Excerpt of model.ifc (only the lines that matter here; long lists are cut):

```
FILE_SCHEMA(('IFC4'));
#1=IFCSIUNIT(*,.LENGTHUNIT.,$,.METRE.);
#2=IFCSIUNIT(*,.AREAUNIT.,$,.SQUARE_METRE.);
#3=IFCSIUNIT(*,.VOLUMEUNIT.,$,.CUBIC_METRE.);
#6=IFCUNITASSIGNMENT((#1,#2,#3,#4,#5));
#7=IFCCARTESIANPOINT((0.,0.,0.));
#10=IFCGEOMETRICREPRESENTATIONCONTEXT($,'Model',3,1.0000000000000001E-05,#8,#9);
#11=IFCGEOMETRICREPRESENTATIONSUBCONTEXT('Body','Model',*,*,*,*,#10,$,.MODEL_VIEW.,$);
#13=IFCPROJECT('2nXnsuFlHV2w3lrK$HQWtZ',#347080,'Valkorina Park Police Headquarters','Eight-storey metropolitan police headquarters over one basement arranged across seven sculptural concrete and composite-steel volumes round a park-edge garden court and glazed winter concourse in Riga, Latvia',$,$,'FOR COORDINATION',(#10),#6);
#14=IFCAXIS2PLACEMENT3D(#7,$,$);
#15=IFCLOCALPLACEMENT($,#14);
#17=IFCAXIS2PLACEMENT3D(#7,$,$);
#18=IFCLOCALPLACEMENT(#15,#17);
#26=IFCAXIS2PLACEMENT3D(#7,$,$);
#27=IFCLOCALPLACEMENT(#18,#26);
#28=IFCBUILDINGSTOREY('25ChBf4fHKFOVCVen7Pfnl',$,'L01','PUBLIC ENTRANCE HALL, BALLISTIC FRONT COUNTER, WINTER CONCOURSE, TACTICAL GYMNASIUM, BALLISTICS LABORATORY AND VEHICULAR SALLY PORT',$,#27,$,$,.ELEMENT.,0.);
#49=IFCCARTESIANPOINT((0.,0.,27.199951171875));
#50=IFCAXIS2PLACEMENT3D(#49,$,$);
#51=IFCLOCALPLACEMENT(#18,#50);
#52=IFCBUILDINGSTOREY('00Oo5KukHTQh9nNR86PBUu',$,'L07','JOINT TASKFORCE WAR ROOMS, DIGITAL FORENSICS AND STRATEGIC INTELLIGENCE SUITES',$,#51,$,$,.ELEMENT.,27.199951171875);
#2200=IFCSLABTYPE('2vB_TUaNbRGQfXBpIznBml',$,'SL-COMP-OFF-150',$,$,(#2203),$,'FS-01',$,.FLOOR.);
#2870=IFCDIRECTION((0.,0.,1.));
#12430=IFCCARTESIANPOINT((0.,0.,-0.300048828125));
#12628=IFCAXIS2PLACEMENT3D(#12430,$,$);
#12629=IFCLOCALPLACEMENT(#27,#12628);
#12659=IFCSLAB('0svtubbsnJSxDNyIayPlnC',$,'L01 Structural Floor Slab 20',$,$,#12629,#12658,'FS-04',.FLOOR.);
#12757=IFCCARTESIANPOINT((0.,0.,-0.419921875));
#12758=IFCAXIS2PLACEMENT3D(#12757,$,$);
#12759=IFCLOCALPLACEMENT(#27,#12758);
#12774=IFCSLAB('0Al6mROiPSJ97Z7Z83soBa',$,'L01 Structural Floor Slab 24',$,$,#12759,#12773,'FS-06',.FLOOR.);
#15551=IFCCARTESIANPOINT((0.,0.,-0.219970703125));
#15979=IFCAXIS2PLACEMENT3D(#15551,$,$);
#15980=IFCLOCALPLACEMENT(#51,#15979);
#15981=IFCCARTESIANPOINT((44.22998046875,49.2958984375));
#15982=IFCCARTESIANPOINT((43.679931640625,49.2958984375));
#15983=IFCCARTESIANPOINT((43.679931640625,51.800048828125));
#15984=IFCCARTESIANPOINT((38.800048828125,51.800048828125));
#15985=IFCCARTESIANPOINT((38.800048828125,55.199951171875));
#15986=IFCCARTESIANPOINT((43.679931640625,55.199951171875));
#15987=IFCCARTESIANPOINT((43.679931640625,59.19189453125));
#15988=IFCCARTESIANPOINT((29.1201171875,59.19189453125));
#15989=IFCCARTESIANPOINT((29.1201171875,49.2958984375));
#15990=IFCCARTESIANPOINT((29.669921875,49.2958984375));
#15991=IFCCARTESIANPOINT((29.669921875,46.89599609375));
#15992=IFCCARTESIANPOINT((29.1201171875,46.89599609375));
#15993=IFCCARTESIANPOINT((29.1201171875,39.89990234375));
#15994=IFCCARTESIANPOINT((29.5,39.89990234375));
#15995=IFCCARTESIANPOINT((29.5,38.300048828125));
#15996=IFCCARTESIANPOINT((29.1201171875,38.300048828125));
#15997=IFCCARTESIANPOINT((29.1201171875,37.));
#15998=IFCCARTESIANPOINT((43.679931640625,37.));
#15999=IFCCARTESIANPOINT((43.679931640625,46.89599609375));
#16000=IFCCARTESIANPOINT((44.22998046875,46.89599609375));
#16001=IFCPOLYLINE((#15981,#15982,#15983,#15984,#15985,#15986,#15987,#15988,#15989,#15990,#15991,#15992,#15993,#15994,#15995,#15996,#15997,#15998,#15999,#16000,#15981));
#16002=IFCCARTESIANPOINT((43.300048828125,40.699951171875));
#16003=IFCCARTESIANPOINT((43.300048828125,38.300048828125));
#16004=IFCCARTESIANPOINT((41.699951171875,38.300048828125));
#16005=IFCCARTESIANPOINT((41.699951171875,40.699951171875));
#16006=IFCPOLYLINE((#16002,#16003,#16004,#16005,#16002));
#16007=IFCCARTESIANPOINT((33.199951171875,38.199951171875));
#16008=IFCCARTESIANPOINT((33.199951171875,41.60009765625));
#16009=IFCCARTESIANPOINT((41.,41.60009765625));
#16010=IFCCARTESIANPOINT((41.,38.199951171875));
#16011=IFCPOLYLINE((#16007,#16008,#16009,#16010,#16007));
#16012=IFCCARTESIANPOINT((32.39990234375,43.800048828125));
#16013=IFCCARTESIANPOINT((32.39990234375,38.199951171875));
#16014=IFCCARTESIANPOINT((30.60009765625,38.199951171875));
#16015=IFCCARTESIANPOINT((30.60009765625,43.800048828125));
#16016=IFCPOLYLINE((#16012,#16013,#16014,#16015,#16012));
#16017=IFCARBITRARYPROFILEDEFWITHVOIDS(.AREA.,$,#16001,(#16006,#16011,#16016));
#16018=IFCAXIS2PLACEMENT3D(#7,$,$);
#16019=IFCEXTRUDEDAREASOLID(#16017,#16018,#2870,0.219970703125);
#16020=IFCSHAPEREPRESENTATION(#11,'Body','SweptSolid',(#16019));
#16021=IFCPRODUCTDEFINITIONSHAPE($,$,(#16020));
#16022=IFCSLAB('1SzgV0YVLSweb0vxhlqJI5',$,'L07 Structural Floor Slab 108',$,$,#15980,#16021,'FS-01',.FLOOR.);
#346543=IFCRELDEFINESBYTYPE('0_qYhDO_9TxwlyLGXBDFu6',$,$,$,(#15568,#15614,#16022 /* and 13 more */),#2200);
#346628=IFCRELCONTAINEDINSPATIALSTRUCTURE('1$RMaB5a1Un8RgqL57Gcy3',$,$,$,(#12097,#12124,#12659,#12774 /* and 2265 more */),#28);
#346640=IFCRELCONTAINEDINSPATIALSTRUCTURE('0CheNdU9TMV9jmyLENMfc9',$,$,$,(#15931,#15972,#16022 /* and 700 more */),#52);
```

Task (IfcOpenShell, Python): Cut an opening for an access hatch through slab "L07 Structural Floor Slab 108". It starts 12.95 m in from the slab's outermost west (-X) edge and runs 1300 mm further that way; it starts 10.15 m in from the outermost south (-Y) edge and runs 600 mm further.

```python
import numpy as np
import ifcopenshell
import ifcopenshell.api.feature
import ifcopenshell.api.geometry
import ifcopenshell.api.root
import ifcopenshell.geom
import ifcopenshell.util.placement
import ifcopenshell.util.representation
import ifcopenshell.util.shape
import ifcopenshell.util.unit

model = ifcopenshell.open("model.ifc")
unit_scale = ifcopenshell.util.unit.calculate_unit_scale(model)
settings = ifcopenshell.geom.settings()


def volume(element):
    """Net volume in cubic metres, openings subtracted."""
    shape = ifcopenshell.geom.create_shape(settings, element)
    return ifcopenshell.util.shape.get_volume(shape.geometry)


slab = model.by_guid("1SzgV0YVLSweb0vxhlqJI5")
before = volume(slab)

# Extent in the slab's own axes, in metres. The edges named are its -X and -Y sides.
slab_shape = ifcopenshell.geom.create_shape(settings, slab)
vertices = ifcopenshell.util.shape.get_vertices(slab_shape.geometry)
x_min, y_min, bottom = vertices.min(axis=0)
top = vertices[:, 2].max()

opening = ifcopenshell.api.root.create_entity(model, ifc_class="IfcOpeningElement", name="Access hatch opening", predefined_type="OPENING")
context = ifcopenshell.util.representation.get_context(model, "Model", "Body", "MODEL_VIEW")
width, depth = 1.3, 0.6
outline = [(0.0, 0.0), (width, 0.0), (width, depth), (0.0, depth), (0.0, 0.0)]
# Overshoot both faces by 50 mm so the cut is clean.
shape = ifcopenshell.api.geometry.add_slab_representation(
    model, context=context, depth=top - bottom + 0.1, polyline=outline
)
ifcopenshell.api.geometry.assign_representation(model, product=opening, representation=shape)

matrix = ifcopenshell.util.placement.get_local_placement(slab.ObjectPlacement)
matrix[:, 3] = matrix @ np.append(np.array([x_min + 12.95, y_min + 10.15, bottom - 0.05]) / unit_scale, 1.0)
ifcopenshell.api.geometry.edit_object_placement(model, product=opening, matrix=matrix, is_si=False)
ifcopenshell.api.feature.add_feature(model, feature=opening, element=slab)

after = volume(slab)

print(f"slab volume {before:.3f} -> {after:.3f} m3")

model.write("model_edited.ifc")
```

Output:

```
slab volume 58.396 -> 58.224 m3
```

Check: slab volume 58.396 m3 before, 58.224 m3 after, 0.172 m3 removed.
